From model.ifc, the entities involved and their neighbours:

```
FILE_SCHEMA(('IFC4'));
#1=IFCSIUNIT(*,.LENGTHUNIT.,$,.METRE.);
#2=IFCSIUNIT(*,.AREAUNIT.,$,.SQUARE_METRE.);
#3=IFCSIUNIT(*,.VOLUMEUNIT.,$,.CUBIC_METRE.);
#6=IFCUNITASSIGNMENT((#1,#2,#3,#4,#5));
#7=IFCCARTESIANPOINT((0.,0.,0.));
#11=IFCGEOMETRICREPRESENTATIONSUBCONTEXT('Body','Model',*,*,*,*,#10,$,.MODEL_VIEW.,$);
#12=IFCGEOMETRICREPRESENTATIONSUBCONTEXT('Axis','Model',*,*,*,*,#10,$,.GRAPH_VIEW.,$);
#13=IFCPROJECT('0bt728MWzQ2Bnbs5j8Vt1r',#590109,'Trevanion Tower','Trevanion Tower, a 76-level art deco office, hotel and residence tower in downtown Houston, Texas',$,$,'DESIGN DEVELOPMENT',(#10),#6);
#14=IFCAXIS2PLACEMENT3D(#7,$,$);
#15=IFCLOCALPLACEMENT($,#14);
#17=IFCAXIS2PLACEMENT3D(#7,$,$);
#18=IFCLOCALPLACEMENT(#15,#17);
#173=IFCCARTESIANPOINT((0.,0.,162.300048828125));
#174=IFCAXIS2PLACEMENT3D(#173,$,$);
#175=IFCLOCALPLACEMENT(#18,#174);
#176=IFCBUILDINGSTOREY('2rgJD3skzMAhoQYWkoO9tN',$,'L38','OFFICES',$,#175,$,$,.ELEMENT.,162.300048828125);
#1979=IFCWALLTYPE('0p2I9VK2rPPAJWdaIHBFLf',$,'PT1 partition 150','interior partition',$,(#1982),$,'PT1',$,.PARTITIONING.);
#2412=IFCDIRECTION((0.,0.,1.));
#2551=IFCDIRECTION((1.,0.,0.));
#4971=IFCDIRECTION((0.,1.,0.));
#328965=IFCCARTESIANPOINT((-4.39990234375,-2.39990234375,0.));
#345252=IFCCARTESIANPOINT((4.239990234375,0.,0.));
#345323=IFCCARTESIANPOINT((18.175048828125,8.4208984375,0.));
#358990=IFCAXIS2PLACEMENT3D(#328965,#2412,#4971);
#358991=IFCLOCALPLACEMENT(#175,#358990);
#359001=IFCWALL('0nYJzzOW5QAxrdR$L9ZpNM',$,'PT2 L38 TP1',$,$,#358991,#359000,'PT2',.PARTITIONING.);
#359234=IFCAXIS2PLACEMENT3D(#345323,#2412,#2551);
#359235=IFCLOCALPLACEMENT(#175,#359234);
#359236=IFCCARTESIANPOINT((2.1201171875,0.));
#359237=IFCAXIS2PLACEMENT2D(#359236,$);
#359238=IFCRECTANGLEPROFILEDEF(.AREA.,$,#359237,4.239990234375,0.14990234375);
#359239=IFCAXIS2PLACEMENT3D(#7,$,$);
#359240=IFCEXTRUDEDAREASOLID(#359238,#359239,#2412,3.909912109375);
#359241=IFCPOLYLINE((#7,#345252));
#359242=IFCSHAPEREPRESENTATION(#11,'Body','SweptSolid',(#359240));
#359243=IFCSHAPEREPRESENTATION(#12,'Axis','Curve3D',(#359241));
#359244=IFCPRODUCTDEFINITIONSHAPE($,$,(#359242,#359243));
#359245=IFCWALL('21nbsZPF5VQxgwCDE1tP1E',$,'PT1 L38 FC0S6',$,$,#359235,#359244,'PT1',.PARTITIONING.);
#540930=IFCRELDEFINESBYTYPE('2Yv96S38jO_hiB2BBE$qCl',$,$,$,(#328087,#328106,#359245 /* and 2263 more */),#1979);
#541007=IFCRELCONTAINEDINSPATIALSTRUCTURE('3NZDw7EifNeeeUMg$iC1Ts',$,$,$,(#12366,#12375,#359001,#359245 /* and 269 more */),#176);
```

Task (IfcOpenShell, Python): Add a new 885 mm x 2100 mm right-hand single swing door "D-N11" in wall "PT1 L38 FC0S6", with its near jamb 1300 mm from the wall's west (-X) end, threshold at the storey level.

```python
import numpy as np
import ifcopenshell
import ifcopenshell.api.feature
import ifcopenshell.api.geometry
import ifcopenshell.api.root
import ifcopenshell.api.spatial
import ifcopenshell.geom
import ifcopenshell.util.element
import ifcopenshell.util.placement
import ifcopenshell.util.representation
import ifcopenshell.util.shape
import ifcopenshell.util.unit

model = ifcopenshell.open("model.ifc")
unit_scale = ifcopenshell.util.unit.calculate_unit_scale(model)
settings = ifcopenshell.geom.settings()


def volume(element):
    """Net volume in cubic metres, openings subtracted."""
    shape = ifcopenshell.geom.create_shape(settings, element)
    return ifcopenshell.util.shape.get_volume(shape.geometry)


wall = model.by_guid("21nbsZPF5VQxgwCDE1tP1E")
storey = ifcopenshell.util.element.get_container(wall, ifc_class="IfcBuildingStorey")
context = ifcopenshell.util.representation.get_context(model, "Model", "Body", "MODEL_VIEW")
before = volume(wall)

width, height, from_end, sill = 0.885, 2.1, 1.3, 0.0  # metres

# The wall runs along its own X axis, and the end named is its -X end.
wall_shape = ifcopenshell.geom.create_shape(settings, wall)
x, y, z = ifcopenshell.util.shape.get_vertices(wall_shape.geometry).T
start = x.min() + from_end
face, thickness = float(y.min()), float(y.max() - y.min())
wall_matrix = ifcopenshell.util.placement.get_local_placement(wall.ObjectPlacement)
level = ifcopenshell.util.placement.get_local_placement(storey.ObjectPlacement)[2, 3]


def in_wall(x, y):
    """Placement at x, y metres in the wall's axes, at sill height."""
    matrix = wall_matrix.copy()
    matrix[:, 3] = wall_matrix @ np.array([x / unit_scale, y / unit_scale, 0.0, 1.0])
    matrix[2, 3] = level + sill / unit_scale
    return matrix


# Opening: a box that overshoots both wall faces by 50 mm.
opening = ifcopenshell.api.root.create_entity(model, ifc_class="IfcOpeningElement", predefined_type="OPENING")
box = ifcopenshell.api.geometry.add_wall_representation(
    model, context=context, length=width, height=height, thickness=thickness + 0.1
)
ifcopenshell.api.geometry.assign_representation(model, product=opening, representation=box)
ifcopenshell.api.geometry.edit_object_placement(model, product=opening, matrix=in_wall(start, face - 0.05), is_si=False)
ifcopenshell.api.feature.add_feature(model, feature=opening, element=wall)

door = ifcopenshell.api.root.create_entity(model, ifc_class="IfcDoor", name="D-N11", predefined_type="DOOR")
door.OverallWidth, door.OverallHeight = width / unit_scale, height / unit_scale
door.OperationType = "SINGLE_SWING_RIGHT"
body = ifcopenshell.api.geometry.add_door_representation(
    model,
    context=context,
    overall_width=door.OverallWidth,
    overall_height=door.OverallHeight,
    operation_type="SINGLE_SWING_RIGHT",
    lining_properties={"LiningDepth": thickness / unit_scale, "ThresholdDepth": thickness / unit_scale},
)
ifcopenshell.api.geometry.assign_representation(model, product=door, representation=body)
ifcopenshell.api.spatial.assign_container(model, products=[door], relating_structure=storey)
ifcopenshell.api.feature.add_filling(model, opening=opening, element=door)

# The lining spans the wall, so the door starts at the wall face.
ifcopenshell.api.geometry.edit_object_placement(model, product=door, matrix=in_wall(start, face), is_si=False)

after = volume(wall)

print(f"wall volume {before:.3f} -> {after:.3f} m3")

model.write("model_v2.ifc")
```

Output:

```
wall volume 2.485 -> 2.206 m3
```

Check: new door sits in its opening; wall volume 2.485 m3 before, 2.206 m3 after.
